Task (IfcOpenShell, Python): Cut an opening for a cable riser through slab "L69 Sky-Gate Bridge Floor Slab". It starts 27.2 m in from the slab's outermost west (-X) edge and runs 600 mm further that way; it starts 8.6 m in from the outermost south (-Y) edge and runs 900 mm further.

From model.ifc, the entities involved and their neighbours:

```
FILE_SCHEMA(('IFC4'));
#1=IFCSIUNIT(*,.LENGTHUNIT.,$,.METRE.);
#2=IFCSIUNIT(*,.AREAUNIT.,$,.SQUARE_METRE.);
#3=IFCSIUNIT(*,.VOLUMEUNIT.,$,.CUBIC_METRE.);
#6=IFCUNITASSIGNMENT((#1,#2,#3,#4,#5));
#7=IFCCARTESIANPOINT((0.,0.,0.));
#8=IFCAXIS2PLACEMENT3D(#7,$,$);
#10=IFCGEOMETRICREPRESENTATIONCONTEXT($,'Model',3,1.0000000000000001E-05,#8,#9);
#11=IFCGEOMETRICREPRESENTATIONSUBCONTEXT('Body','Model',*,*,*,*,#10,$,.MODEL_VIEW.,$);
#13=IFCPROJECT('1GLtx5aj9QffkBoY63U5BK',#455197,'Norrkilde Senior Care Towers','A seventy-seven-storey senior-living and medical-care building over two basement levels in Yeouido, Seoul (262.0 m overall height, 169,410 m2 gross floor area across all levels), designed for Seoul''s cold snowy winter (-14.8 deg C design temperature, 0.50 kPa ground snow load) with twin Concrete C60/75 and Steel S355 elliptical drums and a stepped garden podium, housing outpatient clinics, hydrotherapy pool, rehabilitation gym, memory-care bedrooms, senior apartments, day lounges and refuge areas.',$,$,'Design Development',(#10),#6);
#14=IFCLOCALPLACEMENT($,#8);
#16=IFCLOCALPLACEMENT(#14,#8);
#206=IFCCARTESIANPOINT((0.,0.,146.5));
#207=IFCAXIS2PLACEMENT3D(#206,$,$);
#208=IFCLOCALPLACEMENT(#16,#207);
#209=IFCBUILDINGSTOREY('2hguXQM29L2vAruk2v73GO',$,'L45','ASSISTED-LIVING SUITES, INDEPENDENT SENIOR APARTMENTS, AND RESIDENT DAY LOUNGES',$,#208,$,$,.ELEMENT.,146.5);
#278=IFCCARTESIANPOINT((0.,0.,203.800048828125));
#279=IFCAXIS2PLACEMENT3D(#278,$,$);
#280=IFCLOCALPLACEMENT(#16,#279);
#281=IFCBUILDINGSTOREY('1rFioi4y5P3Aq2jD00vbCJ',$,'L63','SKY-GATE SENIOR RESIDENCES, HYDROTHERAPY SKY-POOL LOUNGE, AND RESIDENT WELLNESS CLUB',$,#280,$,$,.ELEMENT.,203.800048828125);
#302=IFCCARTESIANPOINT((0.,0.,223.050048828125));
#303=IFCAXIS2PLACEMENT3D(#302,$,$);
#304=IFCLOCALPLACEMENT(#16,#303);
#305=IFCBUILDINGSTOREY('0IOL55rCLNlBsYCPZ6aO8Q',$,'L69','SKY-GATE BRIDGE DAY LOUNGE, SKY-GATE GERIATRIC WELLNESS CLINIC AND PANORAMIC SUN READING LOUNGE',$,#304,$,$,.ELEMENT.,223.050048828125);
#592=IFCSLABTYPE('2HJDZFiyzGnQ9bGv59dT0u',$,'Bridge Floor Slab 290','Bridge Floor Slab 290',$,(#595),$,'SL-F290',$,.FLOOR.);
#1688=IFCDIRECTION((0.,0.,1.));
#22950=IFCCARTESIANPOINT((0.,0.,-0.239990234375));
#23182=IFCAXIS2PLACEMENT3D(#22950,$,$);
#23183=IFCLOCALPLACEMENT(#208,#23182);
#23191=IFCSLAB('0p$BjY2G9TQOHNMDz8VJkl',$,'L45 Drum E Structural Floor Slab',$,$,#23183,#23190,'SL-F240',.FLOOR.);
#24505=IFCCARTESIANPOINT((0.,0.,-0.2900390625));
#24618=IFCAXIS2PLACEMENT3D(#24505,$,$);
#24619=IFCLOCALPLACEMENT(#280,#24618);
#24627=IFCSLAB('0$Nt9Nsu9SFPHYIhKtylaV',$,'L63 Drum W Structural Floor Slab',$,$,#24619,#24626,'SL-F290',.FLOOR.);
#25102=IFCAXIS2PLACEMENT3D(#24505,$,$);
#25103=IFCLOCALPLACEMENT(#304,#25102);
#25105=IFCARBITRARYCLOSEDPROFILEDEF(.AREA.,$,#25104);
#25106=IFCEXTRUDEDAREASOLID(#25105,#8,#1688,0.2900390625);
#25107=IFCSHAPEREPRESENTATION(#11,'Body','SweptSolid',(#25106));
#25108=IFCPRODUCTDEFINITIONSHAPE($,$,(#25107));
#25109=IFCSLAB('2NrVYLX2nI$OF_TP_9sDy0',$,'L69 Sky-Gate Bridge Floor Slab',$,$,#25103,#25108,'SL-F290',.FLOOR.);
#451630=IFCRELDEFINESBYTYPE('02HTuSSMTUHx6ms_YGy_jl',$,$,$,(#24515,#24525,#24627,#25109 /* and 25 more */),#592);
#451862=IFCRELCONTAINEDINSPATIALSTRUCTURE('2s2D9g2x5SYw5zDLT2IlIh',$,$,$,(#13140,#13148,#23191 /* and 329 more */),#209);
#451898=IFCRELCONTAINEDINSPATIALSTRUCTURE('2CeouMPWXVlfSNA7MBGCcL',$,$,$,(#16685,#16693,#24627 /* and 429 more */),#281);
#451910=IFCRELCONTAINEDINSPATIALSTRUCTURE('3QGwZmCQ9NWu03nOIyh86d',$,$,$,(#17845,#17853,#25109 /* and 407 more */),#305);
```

```python
import numpy as np
import ifcopenshell
import ifcopenshell.api.feature
import ifcopenshell.api.geometry
import ifcopenshell.api.root
import ifcopenshell.geom
import ifcopenshell.util.placement
import ifcopenshell.util.representation
import ifcopenshell.util.shape
import ifcopenshell.util.unit

model = ifcopenshell.open("model.ifc")
unit_scale = ifcopenshell.util.unit.calculate_unit_scale(model)
settings = ifcopenshell.geom.settings()


def volume(element):
    """Net volume in cubic metres, openings subtracted."""
    shape = ifcopenshell.geom.create_shape(settings, element)
    return ifcopenshell.util.shape.get_volume(shape.geometry)


slab = model.by_guid("2NrVYLX2nI$OF_TP_9sDy0")
before = volume(slab)

# Extent in the slab's own axes, in metres. The edges named are its -X and -Y sides.
slab_shape = ifcopenshell.geom.create_shape(settings, slab)
vertices = ifcopenshell.util.shape.get_vertices(slab_shape.geometry)
x_min, y_min, bottom = vertices.min(axis=0)
top = vertices[:, 2].max()

opening = ifcopenshell.api.root.create_entity(model, ifc_class="IfcOpeningElement", name="Cable riser opening", predefined_type="OPENING")
context = ifcopenshell.util.representation.get_context(model, "Model", "Body", "MODEL_VIEW")
width, depth = 0.6, 0.9
outline = [(0.0, 0.0), (width, 0.0), (width, depth), (0.0, depth), (0.0, 0.0)]
# Overshoot both faces by 50 mm so the cut is clean.
shape = ifcopenshell.api.geometry.add_slab_representation(
    model, context=context, depth=top - bottom + 0.1, polyline=outline
)
ifcopenshell.api.geometry.assign_representation(model, product=opening, representation=shape)

matrix = ifcopenshell.util.placement.get_local_placement(slab.ObjectPlacement)
matrix[:, 3] = matrix @ np.append(np.array([x_min + 27.2, y_min + 8.6, bottom - 0.05]) / unit_scale, 1.0)
ifcopenshell.api.geometry.edit_object_placement(model, product=opening, matrix=matrix, is_si=False)
ifcopenshell.api.feature.add_feature(model, feature=opening, element=slab)

after = volume(slab)

print(f"slab volume {before:.3f} -> {after:.3f} m3")

model.write("model_updated.ifc")
```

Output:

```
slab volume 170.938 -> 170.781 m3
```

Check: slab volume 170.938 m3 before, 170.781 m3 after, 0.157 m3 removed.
